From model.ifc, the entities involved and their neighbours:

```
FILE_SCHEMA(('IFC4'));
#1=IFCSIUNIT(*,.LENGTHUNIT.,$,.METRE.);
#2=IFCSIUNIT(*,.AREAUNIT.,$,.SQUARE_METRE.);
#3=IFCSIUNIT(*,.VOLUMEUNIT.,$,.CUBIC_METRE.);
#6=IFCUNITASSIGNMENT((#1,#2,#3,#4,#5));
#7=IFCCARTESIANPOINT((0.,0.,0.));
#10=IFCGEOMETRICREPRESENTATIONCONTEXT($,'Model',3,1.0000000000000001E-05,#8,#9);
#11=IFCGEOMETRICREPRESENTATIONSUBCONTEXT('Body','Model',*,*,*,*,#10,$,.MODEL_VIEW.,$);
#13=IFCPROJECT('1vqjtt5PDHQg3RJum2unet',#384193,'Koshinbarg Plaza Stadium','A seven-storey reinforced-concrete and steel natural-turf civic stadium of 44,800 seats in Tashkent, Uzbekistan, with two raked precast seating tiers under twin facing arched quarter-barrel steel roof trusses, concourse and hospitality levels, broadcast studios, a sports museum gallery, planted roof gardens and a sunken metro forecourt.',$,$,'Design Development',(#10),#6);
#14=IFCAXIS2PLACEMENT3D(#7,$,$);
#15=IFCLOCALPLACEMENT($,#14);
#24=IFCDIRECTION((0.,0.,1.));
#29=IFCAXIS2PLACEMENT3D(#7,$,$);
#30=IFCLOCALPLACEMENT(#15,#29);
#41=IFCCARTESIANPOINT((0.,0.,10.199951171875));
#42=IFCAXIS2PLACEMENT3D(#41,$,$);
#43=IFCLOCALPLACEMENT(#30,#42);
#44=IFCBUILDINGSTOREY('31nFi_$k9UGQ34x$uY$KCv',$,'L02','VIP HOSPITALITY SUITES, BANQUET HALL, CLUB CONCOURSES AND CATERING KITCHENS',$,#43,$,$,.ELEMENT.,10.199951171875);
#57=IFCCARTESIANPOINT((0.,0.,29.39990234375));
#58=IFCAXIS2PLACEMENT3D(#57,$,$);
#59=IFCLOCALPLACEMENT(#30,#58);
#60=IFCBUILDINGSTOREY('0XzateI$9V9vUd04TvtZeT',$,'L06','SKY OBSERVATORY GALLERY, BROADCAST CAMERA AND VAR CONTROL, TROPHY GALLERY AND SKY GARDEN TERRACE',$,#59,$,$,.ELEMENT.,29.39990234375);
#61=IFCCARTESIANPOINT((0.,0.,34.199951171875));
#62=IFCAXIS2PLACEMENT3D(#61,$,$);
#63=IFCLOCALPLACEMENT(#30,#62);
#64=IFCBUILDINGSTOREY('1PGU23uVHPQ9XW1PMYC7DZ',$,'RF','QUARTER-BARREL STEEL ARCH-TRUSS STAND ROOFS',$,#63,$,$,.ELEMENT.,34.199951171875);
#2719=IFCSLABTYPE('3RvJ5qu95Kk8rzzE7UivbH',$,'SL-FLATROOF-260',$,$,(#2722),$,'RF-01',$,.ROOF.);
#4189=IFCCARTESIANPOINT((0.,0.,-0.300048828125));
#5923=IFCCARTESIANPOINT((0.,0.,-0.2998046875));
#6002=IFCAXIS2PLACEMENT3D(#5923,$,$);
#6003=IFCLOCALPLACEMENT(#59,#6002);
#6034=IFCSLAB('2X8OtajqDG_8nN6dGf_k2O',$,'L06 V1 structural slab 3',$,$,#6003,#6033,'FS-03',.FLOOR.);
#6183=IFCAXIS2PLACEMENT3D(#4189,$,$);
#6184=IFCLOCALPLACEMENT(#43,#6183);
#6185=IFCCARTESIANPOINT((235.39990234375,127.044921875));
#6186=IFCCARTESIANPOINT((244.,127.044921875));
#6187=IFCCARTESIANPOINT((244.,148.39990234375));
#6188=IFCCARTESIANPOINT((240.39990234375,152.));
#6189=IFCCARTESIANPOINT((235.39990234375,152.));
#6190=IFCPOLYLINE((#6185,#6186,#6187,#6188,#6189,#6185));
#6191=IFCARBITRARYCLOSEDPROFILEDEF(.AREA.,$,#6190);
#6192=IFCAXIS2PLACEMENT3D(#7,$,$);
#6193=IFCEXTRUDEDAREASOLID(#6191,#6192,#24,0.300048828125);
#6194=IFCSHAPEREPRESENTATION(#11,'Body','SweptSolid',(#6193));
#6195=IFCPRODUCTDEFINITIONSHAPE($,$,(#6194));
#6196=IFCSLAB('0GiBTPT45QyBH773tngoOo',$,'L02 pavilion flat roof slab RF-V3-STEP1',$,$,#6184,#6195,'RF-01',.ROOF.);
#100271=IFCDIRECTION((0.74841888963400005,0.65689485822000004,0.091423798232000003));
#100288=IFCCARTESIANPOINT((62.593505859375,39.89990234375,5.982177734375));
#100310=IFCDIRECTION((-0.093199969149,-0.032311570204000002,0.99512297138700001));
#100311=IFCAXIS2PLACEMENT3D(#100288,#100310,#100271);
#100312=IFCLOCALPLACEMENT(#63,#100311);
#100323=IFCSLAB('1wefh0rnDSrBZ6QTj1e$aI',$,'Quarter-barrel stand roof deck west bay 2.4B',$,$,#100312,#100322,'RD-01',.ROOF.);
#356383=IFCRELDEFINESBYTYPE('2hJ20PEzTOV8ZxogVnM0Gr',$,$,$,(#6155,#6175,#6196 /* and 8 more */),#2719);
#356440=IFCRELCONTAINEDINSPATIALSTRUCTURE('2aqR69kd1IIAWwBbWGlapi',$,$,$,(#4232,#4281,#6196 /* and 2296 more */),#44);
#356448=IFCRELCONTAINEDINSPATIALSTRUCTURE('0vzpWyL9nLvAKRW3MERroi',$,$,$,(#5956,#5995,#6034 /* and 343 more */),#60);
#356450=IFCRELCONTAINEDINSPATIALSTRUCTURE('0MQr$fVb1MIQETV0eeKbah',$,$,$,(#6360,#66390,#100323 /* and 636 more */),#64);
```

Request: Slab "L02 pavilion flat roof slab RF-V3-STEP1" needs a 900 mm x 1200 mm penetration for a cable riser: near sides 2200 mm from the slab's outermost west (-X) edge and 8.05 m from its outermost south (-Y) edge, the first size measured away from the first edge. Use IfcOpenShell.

```python
import numpy as np
import ifcopenshell
import ifcopenshell.api.feature
import ifcopenshell.api.geometry
import ifcopenshell.api.root
import ifcopenshell.geom
import ifcopenshell.util.placement
import ifcopenshell.util.representation
import ifcopenshell.util.shape
import ifcopenshell.util.unit

model = ifcopenshell.open("model.ifc")
unit_scale = ifcopenshell.util.unit.calculate_unit_scale(model)
settings = ifcopenshell.geom.settings()


def volume(element):
    """Net volume in cubic metres, openings subtracted."""
    shape = ifcopenshell.geom.create_shape(settings, element)
    return ifcopenshell.util.shape.get_volume(shape.geometry)


slab = model.by_guid("0GiBTPT45QyBH773tngoOo")
before = volume(slab)

# Extent in the slab's own axes, in metres. The edges named are its -X and -Y sides.
slab_shape = ifcopenshell.geom.create_shape(settings, slab)
vertices = ifcopenshell.util.shape.get_vertices(slab_shape.geometry)
x_min, y_min, bottom = vertices.min(axis=0)
top = vertices[:, 2].max()

opening = ifcopenshell.api.root.create_entity(model, ifc_class="IfcOpeningElement", name="Cable riser opening", predefined_type="OPENING")
context = ifcopenshell.util.representation.get_context(model, "Model", "Body", "MODEL_VIEW")
width, depth = 0.9, 1.2
outline = [(0.0, 0.0), (width, 0.0), (width, depth), (0.0, depth), (0.0, 0.0)]
# Overshoot both faces by 50 mm so the cut is clean.
shape = ifcopenshell.api.geometry.add_slab_representation(
    model, context=context, depth=top - bottom + 0.1, polyline=outline
)
ifcopenshell.api.geometry.assign_representation(model, product=opening, representation=shape)

matrix = ifcopenshell.util.placement.get_local_placement(slab.ObjectPlacement)
matrix[:, 3] = matrix @ np.append(np.array([x_min + 2.2, y_min + 8.05, bottom - 0.05]) / unit_scale, 1.0)
ifcopenshell.api.geometry.edit_object_placement(model, product=opening, matrix=matrix, is_si=False)
ifcopenshell.api.feature.add_feature(model, feature=opening, element=slab)

after = volume(slab)

print(f"slab volume {before:.3f} -> {after:.3f} m3")

model.write("model-out.ifc")
```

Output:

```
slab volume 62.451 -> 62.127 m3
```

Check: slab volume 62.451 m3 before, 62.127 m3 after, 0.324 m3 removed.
